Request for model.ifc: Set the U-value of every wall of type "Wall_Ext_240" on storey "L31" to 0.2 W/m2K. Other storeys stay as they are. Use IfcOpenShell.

First a look at what the model holds.

```python
import ifcopenshell
import ifcopenshell.util.element

model = ifcopenshell.open("model.ifc")
print(model.schema)
storey = next(s for s in model.by_type("IfcBuildingStorey") if s.Name == "L31")
walls = [e for e in ifcopenshell.util.element.get_decomposition(storey) if e.is_a("IfcWall")]
seen = {}
for e in walls:
    element_type = ifcopenshell.util.element.get_type(e)
    key = (element_type.Name if element_type != e and element_type else None, ifcopenshell.util.element.get_pset(e, "Pset_WallCommon", "ThermalTransmittance"))
    seen[key] = seen.get(key, 0) + 1
for (name, value), count in sorted(seen.items(), key=str):
    print(count, "x", name, "|", value)
```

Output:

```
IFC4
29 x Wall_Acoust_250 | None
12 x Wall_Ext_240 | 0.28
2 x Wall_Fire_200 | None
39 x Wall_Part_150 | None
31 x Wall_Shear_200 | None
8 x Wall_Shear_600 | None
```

```python
import ifcopenshell
import ifcopenshell.api.pset
import ifcopenshell.util.element

model = ifcopenshell.open("model.ifc")

storey = next(s for s in model.by_type("IfcBuildingStorey") if s.Name == "L31")
walls = [e for e in ifcopenshell.util.element.get_decomposition(storey) if e.is_a("IfcWall")]

count = 0
for e in walls:
    element_type = ifcopenshell.util.element.get_type(e)
    if element_type in (None, e) or element_type.Name != "Wall_Ext_240":
        continue
    found = ifcopenshell.util.element.get_pset(e, "Pset_WallCommon", should_inherit=False)
    if found:
        pset = model.by_id(found["id"])
        if len(ifcopenshell.util.element.get_elements_by_pset(pset)) > 1:
            pset = ifcopenshell.api.pset.unshare_pset(model, products=[e], pset=pset)[0]
    else:
        pset = ifcopenshell.api.pset.add_pset(model, product=e, name="Pset_WallCommon")
    ifcopenshell.api.pset.edit_pset(model, pset=pset, properties={"ThermalTransmittance": 0.2})
    count += 1

print(count, "walls updated")

model.write("model_edited.ifc")
```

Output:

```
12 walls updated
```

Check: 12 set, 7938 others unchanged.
